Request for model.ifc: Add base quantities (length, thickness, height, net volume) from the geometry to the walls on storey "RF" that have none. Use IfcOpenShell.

First a look at what the model holds.

```python
import ifcopenshell
import ifcopenshell.util.element
import ifcopenshell.util.unit

model = ifcopenshell.open("model.ifc")
print(model.schema)
for unit_type in ("LENGTHUNIT", "AREAUNIT", "VOLUMEUNIT"):
    print(unit_type, ifcopenshell.util.unit.calculate_unit_scale(model, unit_type))
storey = next(s for s in model.by_type("IfcBuildingStorey") if s.Name == "RF")
walls = [e for e in ifcopenshell.util.element.get_decomposition(storey) if e.is_a("IfcWall")]
for e in sorted(walls, key=lambda e: e.id()):
    print(e.id(), e.is_a(), e.Name, list(ifcopenshell.util.element.get_psets(e, qtos_only=True)), sep=" | ")
```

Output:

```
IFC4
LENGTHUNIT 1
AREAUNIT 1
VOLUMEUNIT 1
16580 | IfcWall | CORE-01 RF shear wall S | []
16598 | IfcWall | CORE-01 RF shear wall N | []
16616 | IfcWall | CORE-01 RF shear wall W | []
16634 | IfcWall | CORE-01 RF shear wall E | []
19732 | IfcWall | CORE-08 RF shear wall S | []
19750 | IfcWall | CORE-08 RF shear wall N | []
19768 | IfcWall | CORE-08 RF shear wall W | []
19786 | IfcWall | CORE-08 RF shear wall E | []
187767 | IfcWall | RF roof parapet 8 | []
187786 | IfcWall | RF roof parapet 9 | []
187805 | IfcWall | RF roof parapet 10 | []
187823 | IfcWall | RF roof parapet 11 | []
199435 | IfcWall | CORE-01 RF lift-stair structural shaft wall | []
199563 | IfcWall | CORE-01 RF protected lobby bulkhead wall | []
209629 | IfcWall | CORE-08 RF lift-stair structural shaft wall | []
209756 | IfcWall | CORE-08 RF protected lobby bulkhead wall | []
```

```python
import ifcopenshell
import ifcopenshell.api.pset
import ifcopenshell.geom
import ifcopenshell.util.element
import ifcopenshell.util.shape
import ifcopenshell.util.unit

model = ifcopenshell.open("model.ifc")
unit_scale = ifcopenshell.util.unit.calculate_unit_scale(model)
volume_scale = ifcopenshell.util.unit.calculate_unit_scale(model, "VOLUMEUNIT")
settings = ifcopenshell.geom.settings()

storey = next(s for s in model.by_type("IfcBuildingStorey") if s.Name == "RF")
walls = [e for e in ifcopenshell.util.element.get_decomposition(storey) if e.is_a("IfcWall")]

for e in sorted(walls, key=lambda e: e.id()):
    if ifcopenshell.util.element.get_psets(e, qtos_only=True, should_inherit=False):
        continue
    # Geometry comes back in metres, in the element's own axes.
    shape = ifcopenshell.geom.create_shape(settings, e)
    values = {
        "Length": ifcopenshell.util.shape.get_x(shape.geometry) / unit_scale,
        "Width": ifcopenshell.util.shape.get_y(shape.geometry) / unit_scale,
        "Height": ifcopenshell.util.shape.get_z(shape.geometry) / unit_scale,
        "NetVolume": ifcopenshell.util.shape.get_volume(shape.geometry) / volume_scale,
    }
    qto = ifcopenshell.api.pset.add_qto(model, product=e, name="Qto_WallBaseQuantities")
    ifcopenshell.api.pset.edit_qto(model, qto=qto, properties=values)
    print(e.id(), {k: round(v, 3) for k, v in values.items()})

model.write("model_rev.ifc")
```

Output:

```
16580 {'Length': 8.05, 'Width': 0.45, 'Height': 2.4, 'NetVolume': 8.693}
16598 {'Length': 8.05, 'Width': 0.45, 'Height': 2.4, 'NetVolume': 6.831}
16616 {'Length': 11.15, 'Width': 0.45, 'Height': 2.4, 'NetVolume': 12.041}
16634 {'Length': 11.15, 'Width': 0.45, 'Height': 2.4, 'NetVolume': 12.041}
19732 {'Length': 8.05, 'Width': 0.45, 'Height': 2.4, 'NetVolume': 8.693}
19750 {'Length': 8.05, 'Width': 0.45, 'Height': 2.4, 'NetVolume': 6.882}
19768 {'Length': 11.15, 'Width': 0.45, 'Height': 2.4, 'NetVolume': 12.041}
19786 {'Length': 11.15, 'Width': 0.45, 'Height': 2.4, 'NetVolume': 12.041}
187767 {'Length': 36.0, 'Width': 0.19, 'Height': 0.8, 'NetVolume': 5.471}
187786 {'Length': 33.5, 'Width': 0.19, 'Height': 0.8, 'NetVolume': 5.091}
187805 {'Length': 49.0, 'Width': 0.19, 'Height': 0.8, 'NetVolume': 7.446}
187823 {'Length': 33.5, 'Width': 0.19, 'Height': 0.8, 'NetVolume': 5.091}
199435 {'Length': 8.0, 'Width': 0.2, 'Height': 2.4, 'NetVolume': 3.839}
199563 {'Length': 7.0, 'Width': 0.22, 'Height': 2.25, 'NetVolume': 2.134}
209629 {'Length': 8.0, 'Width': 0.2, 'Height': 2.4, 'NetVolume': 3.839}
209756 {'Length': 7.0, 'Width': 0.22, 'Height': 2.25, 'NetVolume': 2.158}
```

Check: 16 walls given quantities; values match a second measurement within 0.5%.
